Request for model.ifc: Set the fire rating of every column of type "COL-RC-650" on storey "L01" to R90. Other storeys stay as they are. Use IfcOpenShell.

First a look at what the model holds.

```python
import ifcopenshell
import ifcopenshell.util.element

model = ifcopenshell.open("model.ifc")
print(model.schema)
storey = next(s for s in model.by_type("IfcBuildingStorey") if s.Name == "L01")
columns = [e for e in ifcopenshell.util.element.get_decomposition(storey) if e.is_a("IfcColumn")]
seen = {}
for e in columns:
    element_type = ifcopenshell.util.element.get_type(e)
    key = (element_type.Name if element_type != e and element_type else None, ifcopenshell.util.element.get_pset(e, "Pset_ColumnCommon", "FireRating"))
    seen[key] = seen.get(key, 0) + 1
for (name, value), count in sorted(seen.items(), key=str):
    print(count, "x", name, "|", value)
```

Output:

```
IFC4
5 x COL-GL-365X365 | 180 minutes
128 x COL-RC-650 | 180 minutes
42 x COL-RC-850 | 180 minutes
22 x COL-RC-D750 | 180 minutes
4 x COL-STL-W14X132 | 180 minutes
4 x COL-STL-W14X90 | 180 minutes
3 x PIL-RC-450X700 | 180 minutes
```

```python
import ifcopenshell
import ifcopenshell.api.pset
import ifcopenshell.util.element

model = ifcopenshell.open("model.ifc")

storey = next(s for s in model.by_type("IfcBuildingStorey") if s.Name == "L01")
columns = [e for e in ifcopenshell.util.element.get_decomposition(storey) if e.is_a("IfcColumn")]

count = 0
for e in columns:
    element_type = ifcopenshell.util.element.get_type(e)
    if element_type in (None, e) or element_type.Name != "COL-RC-650":
        continue
    # add_pset returns the element's existing set when there is one.
    pset = ifcopenshell.api.pset.add_pset(model, product=e, name="Pset_ColumnCommon")
    ifcopenshell.api.pset.edit_pset(model, pset=pset, properties={"FireRating": "R90"})
    count += 1

print(count, "columns updated")

model.write("model_v2.ifc")
```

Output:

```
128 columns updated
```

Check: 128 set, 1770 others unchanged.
